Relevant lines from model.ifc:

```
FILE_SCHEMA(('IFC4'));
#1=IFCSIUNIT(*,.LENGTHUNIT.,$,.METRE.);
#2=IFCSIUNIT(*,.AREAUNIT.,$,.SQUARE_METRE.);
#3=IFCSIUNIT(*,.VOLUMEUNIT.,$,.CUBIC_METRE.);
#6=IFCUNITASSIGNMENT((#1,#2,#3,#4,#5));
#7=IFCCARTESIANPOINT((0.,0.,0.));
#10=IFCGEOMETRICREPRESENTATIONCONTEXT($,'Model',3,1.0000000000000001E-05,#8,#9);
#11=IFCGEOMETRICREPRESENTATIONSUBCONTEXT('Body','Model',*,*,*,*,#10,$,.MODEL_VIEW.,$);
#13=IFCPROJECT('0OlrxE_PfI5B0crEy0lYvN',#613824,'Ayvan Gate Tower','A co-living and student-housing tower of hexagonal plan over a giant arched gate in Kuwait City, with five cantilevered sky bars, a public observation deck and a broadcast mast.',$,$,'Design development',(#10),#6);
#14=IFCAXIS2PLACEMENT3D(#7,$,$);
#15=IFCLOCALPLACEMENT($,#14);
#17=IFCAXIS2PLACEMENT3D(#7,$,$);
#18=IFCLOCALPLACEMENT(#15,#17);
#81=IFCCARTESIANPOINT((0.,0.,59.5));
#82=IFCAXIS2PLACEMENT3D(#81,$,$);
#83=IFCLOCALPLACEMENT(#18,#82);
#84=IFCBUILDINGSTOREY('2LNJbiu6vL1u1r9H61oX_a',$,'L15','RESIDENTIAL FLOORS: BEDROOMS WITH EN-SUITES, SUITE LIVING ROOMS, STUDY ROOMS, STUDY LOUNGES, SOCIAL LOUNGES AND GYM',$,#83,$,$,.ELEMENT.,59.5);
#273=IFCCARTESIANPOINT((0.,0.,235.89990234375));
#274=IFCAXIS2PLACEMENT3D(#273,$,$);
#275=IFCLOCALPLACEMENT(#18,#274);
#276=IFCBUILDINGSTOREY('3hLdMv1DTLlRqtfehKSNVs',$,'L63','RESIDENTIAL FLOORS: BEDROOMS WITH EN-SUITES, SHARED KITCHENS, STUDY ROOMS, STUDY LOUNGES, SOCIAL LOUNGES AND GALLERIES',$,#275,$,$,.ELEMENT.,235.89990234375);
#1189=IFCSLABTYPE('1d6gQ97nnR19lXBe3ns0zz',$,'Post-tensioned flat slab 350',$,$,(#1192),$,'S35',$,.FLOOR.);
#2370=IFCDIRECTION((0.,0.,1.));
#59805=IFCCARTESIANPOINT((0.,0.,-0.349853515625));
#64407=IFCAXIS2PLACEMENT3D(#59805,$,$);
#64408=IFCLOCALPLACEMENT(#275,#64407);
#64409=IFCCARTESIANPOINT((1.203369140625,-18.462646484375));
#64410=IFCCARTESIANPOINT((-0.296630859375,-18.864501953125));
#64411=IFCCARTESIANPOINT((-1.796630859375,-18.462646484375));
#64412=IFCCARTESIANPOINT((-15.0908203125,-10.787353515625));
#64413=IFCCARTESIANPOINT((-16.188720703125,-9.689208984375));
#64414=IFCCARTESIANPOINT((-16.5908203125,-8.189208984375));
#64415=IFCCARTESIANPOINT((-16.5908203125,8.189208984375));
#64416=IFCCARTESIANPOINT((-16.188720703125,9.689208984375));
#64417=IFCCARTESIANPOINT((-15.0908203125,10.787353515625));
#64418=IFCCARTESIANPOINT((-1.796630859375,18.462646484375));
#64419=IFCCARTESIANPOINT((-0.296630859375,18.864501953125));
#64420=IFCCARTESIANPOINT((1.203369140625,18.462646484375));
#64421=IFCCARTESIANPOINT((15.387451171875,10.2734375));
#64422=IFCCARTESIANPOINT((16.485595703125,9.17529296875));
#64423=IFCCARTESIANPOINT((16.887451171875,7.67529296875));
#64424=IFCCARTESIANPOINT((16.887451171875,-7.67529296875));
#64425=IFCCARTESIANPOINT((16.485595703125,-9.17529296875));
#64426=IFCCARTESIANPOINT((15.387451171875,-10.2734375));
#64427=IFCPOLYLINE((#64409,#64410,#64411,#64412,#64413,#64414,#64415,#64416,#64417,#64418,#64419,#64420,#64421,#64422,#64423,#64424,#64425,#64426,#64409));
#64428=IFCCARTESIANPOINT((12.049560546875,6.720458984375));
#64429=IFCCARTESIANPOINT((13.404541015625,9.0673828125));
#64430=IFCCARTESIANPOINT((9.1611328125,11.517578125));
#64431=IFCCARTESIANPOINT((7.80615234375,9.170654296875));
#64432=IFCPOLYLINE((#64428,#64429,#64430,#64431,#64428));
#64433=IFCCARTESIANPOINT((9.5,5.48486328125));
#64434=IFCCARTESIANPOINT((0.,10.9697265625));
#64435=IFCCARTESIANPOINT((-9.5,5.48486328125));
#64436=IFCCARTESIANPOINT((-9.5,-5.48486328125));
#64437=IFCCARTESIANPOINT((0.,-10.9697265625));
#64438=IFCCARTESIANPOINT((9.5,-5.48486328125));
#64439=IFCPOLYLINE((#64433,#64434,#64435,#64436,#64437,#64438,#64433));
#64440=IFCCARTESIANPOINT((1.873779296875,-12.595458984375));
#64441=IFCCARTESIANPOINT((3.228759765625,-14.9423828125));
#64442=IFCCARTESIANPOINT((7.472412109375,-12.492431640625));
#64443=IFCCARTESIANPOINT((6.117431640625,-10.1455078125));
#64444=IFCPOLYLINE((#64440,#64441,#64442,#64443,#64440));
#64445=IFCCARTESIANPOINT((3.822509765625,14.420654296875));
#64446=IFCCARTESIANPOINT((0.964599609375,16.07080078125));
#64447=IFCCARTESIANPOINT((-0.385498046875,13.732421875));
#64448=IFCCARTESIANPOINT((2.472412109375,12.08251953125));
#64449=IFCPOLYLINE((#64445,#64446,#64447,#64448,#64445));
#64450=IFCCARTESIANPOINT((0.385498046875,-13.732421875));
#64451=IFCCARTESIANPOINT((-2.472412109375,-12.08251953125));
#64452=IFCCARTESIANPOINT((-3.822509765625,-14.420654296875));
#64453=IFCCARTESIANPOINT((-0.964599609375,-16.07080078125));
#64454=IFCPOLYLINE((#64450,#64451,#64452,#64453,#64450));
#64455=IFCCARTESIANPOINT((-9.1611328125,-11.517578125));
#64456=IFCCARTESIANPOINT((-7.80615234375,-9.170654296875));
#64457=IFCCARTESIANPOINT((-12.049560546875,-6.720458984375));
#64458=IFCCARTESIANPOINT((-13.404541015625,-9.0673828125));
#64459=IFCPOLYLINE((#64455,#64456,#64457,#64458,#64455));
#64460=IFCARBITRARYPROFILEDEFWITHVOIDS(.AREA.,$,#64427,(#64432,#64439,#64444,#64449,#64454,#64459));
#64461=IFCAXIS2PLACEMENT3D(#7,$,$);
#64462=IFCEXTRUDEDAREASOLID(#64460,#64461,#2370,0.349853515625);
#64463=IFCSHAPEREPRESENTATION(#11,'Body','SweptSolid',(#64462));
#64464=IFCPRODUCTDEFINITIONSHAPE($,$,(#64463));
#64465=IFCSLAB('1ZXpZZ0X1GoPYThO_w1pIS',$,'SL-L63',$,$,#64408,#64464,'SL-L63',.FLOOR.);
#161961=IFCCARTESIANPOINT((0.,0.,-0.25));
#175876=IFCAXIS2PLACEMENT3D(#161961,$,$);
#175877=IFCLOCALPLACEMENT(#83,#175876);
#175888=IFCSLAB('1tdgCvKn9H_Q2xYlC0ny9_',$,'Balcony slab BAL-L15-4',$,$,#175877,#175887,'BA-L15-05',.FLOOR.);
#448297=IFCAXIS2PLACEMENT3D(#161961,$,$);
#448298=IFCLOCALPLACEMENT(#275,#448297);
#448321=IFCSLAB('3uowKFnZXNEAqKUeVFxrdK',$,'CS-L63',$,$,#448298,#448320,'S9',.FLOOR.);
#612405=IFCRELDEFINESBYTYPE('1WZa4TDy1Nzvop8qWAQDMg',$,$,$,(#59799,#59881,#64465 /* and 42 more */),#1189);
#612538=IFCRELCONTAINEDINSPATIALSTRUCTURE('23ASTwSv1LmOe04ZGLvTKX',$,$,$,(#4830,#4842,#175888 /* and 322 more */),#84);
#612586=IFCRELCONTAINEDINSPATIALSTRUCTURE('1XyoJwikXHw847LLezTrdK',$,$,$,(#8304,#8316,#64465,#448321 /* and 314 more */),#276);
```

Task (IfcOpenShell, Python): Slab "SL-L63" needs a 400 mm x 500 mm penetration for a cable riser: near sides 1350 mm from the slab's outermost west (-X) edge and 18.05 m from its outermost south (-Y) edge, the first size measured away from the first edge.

```python
import numpy as np
import ifcopenshell
import ifcopenshell.api.feature
import ifcopenshell.api.geometry
import ifcopenshell.api.root
import ifcopenshell.geom
import ifcopenshell.util.placement
import ifcopenshell.util.representation
import ifcopenshell.util.shape
import ifcopenshell.util.unit

model = ifcopenshell.open("model.ifc")
unit_scale = ifcopenshell.util.unit.calculate_unit_scale(model)
settings = ifcopenshell.geom.settings()


def volume(element):
    """Net volume in cubic metres, openings subtracted."""
    shape = ifcopenshell.geom.create_shape(settings, element)
    return ifcopenshell.util.shape.get_volume(shape.geometry)


slab = model.by_guid("1ZXpZZ0X1GoPYThO_w1pIS")
before = volume(slab)

# Extent in the slab's own axes, in metres. The edges named are its -X and -Y sides.
slab_shape = ifcopenshell.geom.create_shape(settings, slab)
vertices = ifcopenshell.util.shape.get_vertices(slab_shape.geometry)
x_min, y_min, bottom = vertices.min(axis=0)
top = vertices[:, 2].max()

opening = ifcopenshell.api.root.create_entity(model, ifc_class="IfcOpeningElement", name="Cable riser opening", predefined_type="OPENING")
context = ifcopenshell.util.representation.get_context(model, "Model", "Body", "MODEL_VIEW")
width, depth = 0.4, 0.5
outline = [(0.0, 0.0), (width, 0.0), (width, depth), (0.0, depth), (0.0, 0.0)]
# Overshoot both faces by 50 mm so the cut is clean.
shape = ifcopenshell.api.geometry.add_slab_representation(
    model, context=context, depth=top - bottom + 0.1, polyline=outline
)
ifcopenshell.api.geometry.assign_representation(model, product=opening, representation=shape)

matrix = ifcopenshell.util.placement.get_local_placement(slab.ObjectPlacement)
matrix[:, 3] = matrix @ np.append(np.array([x_min + 1.35, y_min + 18.05, bottom - 0.05]) / unit_scale, 1.0)
ifcopenshell.api.geometry.edit_object_placement(model, product=opening, matrix=matrix, is_si=False)
ifcopenshell.api.feature.add_feature(model, feature=opening, element=slab)

after = volume(slab)

print(f"slab volume {before:.3f} -> {after:.3f} m3")

model.write("model_edited.ifc")
```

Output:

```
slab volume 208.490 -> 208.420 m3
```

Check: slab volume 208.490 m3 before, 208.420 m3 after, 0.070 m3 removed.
